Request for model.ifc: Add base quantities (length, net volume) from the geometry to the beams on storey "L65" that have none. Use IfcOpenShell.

First a look at what the model holds.

```python
import ifcopenshell
import ifcopenshell.util.element
import ifcopenshell.util.unit

model = ifcopenshell.open("model.ifc")
print(model.schema)
for unit_type in ("LENGTHUNIT", "AREAUNIT", "VOLUMEUNIT"):
    print(unit_type, ifcopenshell.util.unit.calculate_unit_scale(model, unit_type))
storey = next(s for s in model.by_type("IfcBuildingStorey") if s.Name == "L65")
beams = [e for e in ifcopenshell.util.element.get_decomposition(storey) if e.is_a("IfcBeam")]
for e in sorted(beams, key=lambda e: e.id()):
    print(e.id(), e.is_a(), e.Name, list(ifcopenshell.util.element.get_psets(e, qtos_only=True)), sep=" | ")
```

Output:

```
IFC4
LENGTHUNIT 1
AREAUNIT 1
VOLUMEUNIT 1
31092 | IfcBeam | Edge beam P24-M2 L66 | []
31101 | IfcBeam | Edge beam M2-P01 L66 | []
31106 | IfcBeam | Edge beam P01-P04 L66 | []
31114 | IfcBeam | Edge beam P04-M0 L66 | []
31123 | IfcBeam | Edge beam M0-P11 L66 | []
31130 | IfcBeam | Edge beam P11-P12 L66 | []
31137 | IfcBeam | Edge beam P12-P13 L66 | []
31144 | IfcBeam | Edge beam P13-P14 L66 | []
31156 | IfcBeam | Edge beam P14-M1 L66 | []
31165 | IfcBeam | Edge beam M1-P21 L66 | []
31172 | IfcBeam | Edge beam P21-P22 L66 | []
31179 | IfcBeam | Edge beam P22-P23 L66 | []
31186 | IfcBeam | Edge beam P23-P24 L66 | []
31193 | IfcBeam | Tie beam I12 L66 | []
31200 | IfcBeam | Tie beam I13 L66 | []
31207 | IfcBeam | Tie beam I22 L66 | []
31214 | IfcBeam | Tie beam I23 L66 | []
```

```python
import ifcopenshell
import ifcopenshell.api.pset
import ifcopenshell.geom
import ifcopenshell.util.element
import ifcopenshell.util.shape
import ifcopenshell.util.unit

model = ifcopenshell.open("model.ifc")
unit_scale = ifcopenshell.util.unit.calculate_unit_scale(model)
volume_scale = ifcopenshell.util.unit.calculate_unit_scale(model, "VOLUMEUNIT")
settings = ifcopenshell.geom.settings()

storey = next(s for s in model.by_type("IfcBuildingStorey") if s.Name == "L65")
beams = [e for e in ifcopenshell.util.element.get_decomposition(storey) if e.is_a("IfcBeam")]

for e in sorted(beams, key=lambda e: e.id()):
    if ifcopenshell.util.element.get_psets(e, qtos_only=True, should_inherit=False):
        continue
    # Geometry comes back in metres, in the element's own axes.
    shape = ifcopenshell.geom.create_shape(settings, e)
    values = {
        "Length": ifcopenshell.util.shape.get_max_xyz(shape.geometry) / unit_scale,
        "NetVolume": ifcopenshell.util.shape.get_volume(shape.geometry) / volume_scale,
    }
    qto = ifcopenshell.api.pset.add_qto(model, product=e, name="Qto_BeamBaseQuantities")
    ifcopenshell.api.pset.edit_qto(model, qto=qto, properties=values)
    print(e.id(), {k: round(v, 3) for k, v in values.items()})

model.write("model_updated.ifc")
```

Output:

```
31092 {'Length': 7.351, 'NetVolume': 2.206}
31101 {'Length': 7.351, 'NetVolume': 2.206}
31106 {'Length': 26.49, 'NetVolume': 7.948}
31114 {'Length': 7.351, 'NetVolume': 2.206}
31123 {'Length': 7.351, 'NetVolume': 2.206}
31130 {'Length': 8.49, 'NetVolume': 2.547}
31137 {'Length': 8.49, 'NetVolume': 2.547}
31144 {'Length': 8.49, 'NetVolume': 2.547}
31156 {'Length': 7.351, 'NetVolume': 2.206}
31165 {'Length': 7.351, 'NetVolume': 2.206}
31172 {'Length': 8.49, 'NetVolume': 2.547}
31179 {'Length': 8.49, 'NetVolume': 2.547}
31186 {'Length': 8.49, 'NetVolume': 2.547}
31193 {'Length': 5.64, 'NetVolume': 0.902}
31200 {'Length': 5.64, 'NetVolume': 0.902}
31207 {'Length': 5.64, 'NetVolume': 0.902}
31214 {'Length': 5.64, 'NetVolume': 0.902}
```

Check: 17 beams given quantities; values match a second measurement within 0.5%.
